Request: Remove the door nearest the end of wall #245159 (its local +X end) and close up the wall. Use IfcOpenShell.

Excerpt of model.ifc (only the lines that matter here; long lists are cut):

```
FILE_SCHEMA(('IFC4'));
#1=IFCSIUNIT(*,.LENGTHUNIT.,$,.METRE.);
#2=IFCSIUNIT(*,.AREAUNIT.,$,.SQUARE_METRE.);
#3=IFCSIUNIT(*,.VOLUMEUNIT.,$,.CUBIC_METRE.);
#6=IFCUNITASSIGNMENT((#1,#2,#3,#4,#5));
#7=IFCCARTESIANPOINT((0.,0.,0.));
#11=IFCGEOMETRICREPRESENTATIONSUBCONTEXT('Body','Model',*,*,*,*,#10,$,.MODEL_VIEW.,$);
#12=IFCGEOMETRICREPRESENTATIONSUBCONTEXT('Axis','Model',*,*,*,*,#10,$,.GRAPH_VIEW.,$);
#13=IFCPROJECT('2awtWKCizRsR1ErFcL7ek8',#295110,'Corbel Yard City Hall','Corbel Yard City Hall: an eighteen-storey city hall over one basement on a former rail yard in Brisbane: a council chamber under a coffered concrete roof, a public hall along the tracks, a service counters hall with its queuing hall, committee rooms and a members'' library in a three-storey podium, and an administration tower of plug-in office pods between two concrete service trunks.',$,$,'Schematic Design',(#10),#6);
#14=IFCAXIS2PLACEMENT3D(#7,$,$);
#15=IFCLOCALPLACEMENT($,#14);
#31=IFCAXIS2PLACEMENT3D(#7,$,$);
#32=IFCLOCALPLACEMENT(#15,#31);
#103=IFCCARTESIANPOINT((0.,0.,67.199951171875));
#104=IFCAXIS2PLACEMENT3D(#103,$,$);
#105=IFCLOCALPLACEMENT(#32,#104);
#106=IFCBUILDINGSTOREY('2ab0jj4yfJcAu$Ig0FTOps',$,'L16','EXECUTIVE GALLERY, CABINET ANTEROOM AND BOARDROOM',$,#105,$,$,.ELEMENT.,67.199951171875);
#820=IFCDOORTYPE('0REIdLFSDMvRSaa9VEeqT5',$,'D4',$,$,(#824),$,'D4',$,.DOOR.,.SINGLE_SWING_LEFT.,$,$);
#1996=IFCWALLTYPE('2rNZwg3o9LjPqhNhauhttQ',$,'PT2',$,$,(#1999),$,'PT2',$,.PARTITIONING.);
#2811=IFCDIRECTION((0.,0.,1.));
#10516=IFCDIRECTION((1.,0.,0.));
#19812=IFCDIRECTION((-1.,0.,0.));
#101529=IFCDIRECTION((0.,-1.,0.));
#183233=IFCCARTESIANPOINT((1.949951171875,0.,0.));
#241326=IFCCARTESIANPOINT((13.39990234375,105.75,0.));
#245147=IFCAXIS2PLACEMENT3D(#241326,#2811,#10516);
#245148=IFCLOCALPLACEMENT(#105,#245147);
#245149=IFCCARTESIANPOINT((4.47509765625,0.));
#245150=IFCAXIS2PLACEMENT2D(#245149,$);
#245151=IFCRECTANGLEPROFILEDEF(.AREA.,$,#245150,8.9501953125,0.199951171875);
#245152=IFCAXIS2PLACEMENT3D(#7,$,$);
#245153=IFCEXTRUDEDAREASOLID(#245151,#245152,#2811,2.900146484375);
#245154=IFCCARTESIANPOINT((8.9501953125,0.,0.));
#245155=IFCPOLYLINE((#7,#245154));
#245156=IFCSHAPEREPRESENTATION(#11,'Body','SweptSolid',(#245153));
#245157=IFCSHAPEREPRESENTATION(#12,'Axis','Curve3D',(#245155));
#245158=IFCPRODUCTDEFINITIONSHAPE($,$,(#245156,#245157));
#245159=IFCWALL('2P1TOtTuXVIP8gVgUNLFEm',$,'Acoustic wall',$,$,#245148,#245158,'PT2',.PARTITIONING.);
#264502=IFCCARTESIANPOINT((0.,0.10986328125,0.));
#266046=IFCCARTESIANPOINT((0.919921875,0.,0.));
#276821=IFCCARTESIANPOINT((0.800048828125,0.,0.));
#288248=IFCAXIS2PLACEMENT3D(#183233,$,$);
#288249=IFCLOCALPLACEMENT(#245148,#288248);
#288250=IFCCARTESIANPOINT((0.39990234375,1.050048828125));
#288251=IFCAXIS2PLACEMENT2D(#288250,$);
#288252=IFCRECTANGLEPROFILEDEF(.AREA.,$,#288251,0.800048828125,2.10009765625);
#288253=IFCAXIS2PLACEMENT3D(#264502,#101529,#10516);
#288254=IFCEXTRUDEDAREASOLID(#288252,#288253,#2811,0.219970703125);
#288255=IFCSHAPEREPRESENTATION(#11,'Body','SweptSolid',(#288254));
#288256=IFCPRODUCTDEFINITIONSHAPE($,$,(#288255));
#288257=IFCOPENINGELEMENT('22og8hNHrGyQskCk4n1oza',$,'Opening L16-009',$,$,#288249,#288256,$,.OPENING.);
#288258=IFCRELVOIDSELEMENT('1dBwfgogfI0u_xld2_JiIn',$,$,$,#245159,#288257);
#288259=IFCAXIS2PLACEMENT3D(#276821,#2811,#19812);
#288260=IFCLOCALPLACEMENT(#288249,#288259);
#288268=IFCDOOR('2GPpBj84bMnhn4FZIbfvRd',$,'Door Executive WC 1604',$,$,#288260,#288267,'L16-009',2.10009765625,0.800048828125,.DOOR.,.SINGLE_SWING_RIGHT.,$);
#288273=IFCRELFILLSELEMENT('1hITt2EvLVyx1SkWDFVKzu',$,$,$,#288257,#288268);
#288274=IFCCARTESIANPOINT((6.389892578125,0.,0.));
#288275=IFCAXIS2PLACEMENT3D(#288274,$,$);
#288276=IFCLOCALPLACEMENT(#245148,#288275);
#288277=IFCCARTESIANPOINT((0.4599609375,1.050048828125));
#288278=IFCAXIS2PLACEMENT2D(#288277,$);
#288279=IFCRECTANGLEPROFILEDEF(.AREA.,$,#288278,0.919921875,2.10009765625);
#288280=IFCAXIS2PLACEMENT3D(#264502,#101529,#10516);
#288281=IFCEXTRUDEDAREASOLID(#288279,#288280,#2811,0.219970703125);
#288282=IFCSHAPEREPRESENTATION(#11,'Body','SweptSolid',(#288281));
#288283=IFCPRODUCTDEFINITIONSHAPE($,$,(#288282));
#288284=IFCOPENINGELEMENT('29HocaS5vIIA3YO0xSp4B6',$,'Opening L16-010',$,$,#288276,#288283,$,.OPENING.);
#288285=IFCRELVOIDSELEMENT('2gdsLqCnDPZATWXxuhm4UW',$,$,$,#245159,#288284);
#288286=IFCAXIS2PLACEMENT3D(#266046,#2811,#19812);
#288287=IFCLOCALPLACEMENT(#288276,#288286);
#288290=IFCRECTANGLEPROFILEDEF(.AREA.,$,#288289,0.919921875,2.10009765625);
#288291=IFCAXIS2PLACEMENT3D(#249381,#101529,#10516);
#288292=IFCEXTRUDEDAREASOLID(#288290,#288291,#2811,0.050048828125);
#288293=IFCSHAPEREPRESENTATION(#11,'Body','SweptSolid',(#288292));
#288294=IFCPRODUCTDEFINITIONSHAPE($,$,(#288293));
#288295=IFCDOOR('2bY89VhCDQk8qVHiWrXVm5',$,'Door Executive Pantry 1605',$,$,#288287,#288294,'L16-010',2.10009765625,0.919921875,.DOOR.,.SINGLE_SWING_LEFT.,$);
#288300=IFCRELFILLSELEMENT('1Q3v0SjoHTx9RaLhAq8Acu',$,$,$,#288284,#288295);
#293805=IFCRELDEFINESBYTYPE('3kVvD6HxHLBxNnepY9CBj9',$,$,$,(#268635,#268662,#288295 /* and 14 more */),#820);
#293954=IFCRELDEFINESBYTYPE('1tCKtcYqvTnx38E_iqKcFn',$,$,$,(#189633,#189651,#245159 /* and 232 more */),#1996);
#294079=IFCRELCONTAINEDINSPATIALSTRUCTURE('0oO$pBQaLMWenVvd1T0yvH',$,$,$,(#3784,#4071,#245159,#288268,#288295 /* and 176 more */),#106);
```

```python
import ifcopenshell
import ifcopenshell.api.feature
import ifcopenshell.api.root
import ifcopenshell.geom
import ifcopenshell.util.shape

model = ifcopenshell.open("model.ifc")
settings = ifcopenshell.geom.settings()


def volume(element):
    """Net volume in cubic metres, openings subtracted."""
    shape = ifcopenshell.geom.create_shape(settings, element)
    return ifcopenshell.util.shape.get_volume(shape.geometry)


door = model.by_guid("2bY89VhCDQk8qVHiWrXVm5")
opening = door.FillsVoids[0].RelatingOpeningElement
wall = opening.VoidsElements[0].RelatingBuildingElement
before = volume(wall)

ifcopenshell.api.root.remove_product(model, product=door)
ifcopenshell.api.feature.remove_feature(model, feature=opening)

after = volume(wall)

print(f"wall volume {before:.3f} -> {after:.3f} m3")

model.write("model_updated.ifc")
```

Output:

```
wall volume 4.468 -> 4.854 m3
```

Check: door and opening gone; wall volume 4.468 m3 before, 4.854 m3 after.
